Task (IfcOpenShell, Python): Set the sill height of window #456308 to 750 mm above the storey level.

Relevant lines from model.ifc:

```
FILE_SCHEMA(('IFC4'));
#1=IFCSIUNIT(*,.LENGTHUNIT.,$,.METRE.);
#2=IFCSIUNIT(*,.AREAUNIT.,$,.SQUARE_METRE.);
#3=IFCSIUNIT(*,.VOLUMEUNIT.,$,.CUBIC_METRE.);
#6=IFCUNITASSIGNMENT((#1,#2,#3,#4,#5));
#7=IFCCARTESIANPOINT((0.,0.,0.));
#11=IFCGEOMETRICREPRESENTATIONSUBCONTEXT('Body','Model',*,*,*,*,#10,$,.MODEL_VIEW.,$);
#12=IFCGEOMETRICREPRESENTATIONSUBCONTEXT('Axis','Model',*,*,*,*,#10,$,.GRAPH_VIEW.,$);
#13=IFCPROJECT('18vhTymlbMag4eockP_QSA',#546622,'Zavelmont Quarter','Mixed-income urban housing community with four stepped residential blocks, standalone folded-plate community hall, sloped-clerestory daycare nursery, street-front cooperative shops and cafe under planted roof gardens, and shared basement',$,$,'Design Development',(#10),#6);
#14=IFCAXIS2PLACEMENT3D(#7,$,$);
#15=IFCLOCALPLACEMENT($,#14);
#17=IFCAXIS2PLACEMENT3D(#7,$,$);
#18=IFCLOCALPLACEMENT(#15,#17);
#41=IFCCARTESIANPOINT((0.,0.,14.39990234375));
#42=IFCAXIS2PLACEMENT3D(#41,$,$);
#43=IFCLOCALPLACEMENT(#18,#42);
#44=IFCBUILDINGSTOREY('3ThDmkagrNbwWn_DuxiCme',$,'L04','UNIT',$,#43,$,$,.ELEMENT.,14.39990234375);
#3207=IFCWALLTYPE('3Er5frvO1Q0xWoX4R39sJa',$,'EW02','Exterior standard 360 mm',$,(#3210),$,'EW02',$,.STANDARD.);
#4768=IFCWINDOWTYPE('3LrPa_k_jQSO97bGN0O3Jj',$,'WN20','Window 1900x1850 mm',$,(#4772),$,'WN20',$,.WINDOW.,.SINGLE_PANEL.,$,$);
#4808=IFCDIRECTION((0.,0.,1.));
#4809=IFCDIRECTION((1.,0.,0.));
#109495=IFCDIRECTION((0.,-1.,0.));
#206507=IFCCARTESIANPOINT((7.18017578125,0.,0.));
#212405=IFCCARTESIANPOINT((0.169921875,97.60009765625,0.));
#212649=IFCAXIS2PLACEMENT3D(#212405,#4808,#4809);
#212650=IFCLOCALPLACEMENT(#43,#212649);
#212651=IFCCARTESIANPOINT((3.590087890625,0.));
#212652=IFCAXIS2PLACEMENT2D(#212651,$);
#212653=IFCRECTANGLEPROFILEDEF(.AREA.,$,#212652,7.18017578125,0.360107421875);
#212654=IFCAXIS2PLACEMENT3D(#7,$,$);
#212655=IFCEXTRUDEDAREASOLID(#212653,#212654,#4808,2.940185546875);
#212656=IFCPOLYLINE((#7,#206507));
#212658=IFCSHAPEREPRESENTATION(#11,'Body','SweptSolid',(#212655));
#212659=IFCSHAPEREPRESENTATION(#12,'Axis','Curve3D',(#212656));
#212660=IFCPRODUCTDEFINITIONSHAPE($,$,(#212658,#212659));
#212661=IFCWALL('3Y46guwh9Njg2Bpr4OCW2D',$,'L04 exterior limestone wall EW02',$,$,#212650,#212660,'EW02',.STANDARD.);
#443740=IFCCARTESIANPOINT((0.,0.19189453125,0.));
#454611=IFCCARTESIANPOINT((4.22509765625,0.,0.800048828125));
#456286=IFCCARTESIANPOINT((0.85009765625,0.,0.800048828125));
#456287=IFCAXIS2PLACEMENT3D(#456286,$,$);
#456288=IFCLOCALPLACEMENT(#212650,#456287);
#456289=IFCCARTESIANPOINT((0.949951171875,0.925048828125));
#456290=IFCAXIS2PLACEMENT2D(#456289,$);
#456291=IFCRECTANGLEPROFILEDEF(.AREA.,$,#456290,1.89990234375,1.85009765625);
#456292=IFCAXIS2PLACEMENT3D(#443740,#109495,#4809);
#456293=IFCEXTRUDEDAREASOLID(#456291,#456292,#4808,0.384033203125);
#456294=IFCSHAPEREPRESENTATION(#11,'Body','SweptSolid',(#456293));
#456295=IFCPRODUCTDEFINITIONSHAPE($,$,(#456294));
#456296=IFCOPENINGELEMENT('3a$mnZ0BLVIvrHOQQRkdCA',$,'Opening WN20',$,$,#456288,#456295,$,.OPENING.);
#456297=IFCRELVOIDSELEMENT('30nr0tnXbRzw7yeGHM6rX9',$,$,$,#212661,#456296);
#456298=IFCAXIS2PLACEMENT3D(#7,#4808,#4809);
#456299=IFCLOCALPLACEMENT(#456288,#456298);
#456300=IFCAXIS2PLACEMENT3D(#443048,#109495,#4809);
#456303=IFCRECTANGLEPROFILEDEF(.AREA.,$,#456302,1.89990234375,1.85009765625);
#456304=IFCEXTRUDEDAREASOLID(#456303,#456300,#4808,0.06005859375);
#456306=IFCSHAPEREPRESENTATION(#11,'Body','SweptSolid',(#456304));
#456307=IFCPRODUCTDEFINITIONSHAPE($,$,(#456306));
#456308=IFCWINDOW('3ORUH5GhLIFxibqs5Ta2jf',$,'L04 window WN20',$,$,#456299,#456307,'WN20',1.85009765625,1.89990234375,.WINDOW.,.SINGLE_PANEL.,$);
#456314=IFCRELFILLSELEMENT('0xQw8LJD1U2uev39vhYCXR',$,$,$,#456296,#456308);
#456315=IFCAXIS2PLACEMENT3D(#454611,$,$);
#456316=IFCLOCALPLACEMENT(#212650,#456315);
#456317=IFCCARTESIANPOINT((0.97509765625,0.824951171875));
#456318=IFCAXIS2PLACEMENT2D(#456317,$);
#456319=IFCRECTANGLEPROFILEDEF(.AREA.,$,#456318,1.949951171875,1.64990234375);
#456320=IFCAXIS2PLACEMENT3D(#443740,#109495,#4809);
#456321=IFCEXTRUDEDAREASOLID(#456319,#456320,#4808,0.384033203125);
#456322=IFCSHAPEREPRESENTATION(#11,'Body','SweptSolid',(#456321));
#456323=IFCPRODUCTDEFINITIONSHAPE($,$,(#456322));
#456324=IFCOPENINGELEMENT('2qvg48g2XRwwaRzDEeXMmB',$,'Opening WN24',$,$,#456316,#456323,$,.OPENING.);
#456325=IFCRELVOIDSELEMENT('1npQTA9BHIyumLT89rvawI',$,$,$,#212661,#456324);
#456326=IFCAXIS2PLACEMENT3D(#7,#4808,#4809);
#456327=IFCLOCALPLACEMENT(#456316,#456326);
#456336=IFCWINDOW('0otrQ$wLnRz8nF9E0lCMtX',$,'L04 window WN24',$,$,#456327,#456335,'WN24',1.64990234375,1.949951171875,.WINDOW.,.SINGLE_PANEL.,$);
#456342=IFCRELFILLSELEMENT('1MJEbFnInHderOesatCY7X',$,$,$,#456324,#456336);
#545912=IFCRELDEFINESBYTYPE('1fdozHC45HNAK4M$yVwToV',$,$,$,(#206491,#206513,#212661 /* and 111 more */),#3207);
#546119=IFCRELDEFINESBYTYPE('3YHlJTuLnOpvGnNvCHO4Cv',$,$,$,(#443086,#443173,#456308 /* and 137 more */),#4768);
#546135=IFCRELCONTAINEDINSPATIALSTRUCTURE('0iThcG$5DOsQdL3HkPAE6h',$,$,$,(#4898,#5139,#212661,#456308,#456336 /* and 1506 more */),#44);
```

```python
import numpy as np
import ifcopenshell
import ifcopenshell.api.geometry
import ifcopenshell.geom
import ifcopenshell.util.element
import ifcopenshell.util.placement
import ifcopenshell.util.shape
import ifcopenshell.util.unit

model = ifcopenshell.open("model.ifc")
unit_scale = ifcopenshell.util.unit.calculate_unit_scale(model)

window = model.by_id(456308)
opening = window.FillsVoids[0].RelatingOpeningElement
storey = ifcopenshell.util.element.get_container(window, ifc_class="IfcBuildingStorey")
level = ifcopenshell.util.placement.get_local_placement(storey.ObjectPlacement)[2, 3]

# The opening's origin need not be at the sill, so measure its lowest point.
shape = ifcopenshell.geom.create_shape(ifcopenshell.geom.settings(), opening)
bottom = ifcopenshell.util.shape.get_shape_bottom_elevation(shape, shape.geometry) / unit_scale
dz = level + 0.75 - bottom

shift = np.array([0.0, 0.0, dz])
# The window is placed relative to its opening, so it follows when the opening moves.
matrix = ifcopenshell.util.placement.get_local_placement(opening.ObjectPlacement)
matrix[:3, 3] += shift
ifcopenshell.api.geometry.edit_object_placement(
    model, product=opening, matrix=matrix, is_si=False, should_transform_children=True
)

print(f"moved by {dz * unit_scale:+.3f} m")

model.write("model_edited.ifc")
```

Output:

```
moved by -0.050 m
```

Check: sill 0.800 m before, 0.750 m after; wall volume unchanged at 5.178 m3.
